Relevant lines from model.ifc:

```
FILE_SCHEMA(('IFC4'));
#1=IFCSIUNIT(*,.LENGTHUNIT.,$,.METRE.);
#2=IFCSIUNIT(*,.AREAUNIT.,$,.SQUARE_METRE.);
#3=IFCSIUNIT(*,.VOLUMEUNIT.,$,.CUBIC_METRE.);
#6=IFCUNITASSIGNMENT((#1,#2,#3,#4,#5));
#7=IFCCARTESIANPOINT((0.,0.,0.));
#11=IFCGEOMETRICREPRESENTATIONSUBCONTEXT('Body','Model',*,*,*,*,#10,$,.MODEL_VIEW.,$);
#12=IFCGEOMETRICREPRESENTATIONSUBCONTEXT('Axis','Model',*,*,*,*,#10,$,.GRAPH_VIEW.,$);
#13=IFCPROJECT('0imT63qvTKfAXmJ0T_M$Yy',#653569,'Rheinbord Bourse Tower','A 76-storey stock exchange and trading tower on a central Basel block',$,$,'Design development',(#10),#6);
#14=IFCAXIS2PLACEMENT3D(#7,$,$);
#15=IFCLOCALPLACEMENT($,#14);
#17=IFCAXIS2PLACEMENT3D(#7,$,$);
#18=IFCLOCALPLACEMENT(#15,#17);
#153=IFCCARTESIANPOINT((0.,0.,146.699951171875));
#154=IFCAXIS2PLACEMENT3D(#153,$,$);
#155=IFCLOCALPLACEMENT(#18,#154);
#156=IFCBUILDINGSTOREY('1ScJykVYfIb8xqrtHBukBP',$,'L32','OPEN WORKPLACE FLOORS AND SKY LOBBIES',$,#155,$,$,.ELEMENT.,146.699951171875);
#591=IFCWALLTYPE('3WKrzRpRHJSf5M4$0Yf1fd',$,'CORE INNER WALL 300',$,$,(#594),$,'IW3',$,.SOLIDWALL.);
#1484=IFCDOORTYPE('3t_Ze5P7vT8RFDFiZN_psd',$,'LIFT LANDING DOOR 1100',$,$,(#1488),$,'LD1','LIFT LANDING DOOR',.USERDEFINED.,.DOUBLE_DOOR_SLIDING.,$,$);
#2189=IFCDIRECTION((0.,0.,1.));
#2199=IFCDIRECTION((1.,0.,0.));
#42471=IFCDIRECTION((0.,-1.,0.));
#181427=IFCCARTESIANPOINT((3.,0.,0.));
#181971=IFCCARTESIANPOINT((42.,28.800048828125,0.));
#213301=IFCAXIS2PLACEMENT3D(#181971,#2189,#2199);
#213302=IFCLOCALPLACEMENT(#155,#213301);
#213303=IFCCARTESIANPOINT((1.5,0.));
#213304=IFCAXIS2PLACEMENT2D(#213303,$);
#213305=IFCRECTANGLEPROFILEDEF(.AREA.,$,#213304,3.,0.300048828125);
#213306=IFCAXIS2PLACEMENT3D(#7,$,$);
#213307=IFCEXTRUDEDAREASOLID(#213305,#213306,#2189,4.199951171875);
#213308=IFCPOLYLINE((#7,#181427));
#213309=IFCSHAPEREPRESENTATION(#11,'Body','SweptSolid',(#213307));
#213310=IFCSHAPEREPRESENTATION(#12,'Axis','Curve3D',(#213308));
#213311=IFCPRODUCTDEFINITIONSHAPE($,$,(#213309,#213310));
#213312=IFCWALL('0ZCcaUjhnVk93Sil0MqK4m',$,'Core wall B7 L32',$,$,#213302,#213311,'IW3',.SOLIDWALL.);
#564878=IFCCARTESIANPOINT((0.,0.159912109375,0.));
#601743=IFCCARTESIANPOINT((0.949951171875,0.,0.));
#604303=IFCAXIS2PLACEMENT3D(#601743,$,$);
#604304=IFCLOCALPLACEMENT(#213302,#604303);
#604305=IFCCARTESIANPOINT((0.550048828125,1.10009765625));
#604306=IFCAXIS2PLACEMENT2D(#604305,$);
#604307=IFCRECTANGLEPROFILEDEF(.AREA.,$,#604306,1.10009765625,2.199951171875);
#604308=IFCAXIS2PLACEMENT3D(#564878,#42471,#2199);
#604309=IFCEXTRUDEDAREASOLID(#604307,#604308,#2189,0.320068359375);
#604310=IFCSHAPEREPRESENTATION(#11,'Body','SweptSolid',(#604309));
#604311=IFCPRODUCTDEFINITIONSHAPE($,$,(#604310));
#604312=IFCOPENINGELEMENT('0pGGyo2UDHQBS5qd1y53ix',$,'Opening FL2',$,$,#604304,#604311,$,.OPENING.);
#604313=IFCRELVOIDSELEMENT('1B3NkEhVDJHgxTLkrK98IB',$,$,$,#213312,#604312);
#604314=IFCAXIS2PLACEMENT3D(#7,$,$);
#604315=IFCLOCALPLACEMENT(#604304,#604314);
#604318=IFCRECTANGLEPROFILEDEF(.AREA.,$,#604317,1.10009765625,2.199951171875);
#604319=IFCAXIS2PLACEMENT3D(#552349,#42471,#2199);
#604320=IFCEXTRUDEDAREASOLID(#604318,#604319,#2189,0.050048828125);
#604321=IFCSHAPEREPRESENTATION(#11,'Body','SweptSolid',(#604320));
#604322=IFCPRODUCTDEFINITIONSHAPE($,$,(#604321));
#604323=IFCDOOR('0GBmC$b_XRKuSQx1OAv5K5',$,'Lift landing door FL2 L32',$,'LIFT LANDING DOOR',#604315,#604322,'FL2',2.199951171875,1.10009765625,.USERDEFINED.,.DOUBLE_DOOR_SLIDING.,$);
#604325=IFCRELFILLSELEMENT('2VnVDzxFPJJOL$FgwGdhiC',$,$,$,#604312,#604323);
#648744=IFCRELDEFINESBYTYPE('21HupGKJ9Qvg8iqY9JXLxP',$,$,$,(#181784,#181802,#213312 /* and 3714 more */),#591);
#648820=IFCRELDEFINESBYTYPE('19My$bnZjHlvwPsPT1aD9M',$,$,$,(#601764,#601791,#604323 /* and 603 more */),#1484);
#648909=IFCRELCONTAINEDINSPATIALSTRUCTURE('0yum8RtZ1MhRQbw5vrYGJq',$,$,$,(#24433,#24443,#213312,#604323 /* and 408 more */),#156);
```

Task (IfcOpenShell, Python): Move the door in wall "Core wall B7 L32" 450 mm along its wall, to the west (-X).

```python
import ifcopenshell
import ifcopenshell.api.geometry
import ifcopenshell.util.placement
import ifcopenshell.util.unit

model = ifcopenshell.open("model.ifc")
unit_scale = ifcopenshell.util.unit.calculate_unit_scale(model)

door = model.by_guid("0GBmC$b_XRKuSQx1OAv5K5")
opening = door.FillsVoids[0].RelatingOpeningElement
wall = opening.VoidsElements[0].RelatingBuildingElement

wall_matrix = ifcopenshell.util.placement.get_local_placement(wall.ObjectPlacement)
shift = wall_matrix[:3, 0] * -0.45 / unit_scale
before = ifcopenshell.util.placement.get_local_placement(door.ObjectPlacement)[:3, 3].copy()

# The door is placed relative to its opening, so it follows when the opening moves.
matrix = ifcopenshell.util.placement.get_local_placement(opening.ObjectPlacement)
matrix[:3, 3] += shift
ifcopenshell.api.geometry.edit_object_placement(
    model, product=opening, matrix=matrix, is_si=False, should_transform_children=True
)

after = ifcopenshell.util.placement.get_local_placement(door.ObjectPlacement)[:3, 3]
print("door moved by", (after - before).round(3) + 0.0)

model.write("model-out.ifc")
```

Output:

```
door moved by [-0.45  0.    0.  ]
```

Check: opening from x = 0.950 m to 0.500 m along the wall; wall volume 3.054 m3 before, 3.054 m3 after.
